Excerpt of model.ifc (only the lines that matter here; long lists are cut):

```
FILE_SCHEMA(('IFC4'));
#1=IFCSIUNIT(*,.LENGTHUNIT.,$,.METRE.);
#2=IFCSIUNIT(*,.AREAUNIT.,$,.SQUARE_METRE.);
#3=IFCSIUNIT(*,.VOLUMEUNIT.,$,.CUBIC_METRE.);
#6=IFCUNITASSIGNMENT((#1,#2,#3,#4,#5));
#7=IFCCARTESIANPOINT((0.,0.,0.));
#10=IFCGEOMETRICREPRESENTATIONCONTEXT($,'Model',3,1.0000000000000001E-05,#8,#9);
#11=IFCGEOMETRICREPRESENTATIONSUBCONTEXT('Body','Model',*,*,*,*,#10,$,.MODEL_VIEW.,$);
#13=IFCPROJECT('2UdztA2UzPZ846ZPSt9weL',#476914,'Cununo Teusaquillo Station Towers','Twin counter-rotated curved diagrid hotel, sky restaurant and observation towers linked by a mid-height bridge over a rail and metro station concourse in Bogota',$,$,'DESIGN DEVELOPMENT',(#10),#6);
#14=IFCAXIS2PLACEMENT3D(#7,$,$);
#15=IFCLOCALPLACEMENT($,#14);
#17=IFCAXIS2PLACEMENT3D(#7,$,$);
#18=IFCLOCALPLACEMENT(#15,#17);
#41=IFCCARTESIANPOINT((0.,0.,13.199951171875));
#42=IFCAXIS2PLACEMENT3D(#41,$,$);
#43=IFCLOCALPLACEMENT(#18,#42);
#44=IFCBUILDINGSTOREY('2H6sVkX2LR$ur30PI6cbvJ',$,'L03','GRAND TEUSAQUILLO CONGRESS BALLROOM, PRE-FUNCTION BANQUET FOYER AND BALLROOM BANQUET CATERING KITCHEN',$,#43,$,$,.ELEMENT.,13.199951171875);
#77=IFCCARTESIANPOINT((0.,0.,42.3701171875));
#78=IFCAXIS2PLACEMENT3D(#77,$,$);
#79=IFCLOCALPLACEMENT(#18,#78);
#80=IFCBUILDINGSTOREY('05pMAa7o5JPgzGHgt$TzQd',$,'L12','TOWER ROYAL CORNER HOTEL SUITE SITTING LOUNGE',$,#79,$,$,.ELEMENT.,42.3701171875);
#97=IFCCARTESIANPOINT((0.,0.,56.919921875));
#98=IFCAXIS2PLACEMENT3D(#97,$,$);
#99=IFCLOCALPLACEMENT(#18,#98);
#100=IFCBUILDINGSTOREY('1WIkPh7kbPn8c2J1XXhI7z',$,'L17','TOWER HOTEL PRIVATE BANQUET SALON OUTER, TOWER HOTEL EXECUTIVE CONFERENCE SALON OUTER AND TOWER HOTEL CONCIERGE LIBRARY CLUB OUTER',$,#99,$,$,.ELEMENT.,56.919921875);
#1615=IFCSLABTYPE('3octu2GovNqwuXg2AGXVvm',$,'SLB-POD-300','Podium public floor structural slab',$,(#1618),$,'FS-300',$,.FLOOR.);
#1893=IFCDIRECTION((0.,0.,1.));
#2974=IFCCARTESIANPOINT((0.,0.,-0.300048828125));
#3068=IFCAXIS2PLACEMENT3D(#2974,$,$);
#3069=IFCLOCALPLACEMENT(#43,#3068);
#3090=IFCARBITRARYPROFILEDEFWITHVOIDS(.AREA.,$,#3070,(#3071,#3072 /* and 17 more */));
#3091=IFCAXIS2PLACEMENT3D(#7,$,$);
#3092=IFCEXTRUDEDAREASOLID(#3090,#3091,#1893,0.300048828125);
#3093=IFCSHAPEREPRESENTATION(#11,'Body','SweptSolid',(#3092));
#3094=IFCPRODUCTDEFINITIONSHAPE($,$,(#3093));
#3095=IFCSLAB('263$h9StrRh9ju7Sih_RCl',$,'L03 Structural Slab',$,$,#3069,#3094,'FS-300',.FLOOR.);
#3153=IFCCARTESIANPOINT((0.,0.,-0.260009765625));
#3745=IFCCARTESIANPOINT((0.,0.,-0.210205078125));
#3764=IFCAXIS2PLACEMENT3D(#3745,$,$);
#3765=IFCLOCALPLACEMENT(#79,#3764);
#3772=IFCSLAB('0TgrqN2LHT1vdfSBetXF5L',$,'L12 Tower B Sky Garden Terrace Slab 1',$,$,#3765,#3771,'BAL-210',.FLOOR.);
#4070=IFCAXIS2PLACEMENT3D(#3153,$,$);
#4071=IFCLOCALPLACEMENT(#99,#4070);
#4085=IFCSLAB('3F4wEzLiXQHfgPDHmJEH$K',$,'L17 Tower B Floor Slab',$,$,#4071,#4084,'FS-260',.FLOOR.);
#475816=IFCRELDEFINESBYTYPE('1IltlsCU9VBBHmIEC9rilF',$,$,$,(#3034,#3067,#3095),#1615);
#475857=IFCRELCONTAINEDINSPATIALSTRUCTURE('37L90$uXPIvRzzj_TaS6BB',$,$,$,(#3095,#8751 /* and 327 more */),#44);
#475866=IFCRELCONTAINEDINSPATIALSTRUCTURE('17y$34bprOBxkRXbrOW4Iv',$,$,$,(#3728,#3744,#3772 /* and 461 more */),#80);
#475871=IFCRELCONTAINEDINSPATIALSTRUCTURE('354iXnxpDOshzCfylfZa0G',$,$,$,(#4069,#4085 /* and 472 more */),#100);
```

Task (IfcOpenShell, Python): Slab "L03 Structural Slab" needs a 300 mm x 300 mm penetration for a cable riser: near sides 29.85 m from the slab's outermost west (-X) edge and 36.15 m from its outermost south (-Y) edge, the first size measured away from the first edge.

```python
import numpy as np
import ifcopenshell
import ifcopenshell.api.feature
import ifcopenshell.api.geometry
import ifcopenshell.api.root
import ifcopenshell.geom
import ifcopenshell.util.placement
import ifcopenshell.util.representation
import ifcopenshell.util.shape
import ifcopenshell.util.unit

model = ifcopenshell.open("model.ifc")
unit_scale = ifcopenshell.util.unit.calculate_unit_scale(model)
settings = ifcopenshell.geom.settings()


def volume(element):
    """Net volume in cubic metres, openings subtracted."""
    shape = ifcopenshell.geom.create_shape(settings, element)
    return ifcopenshell.util.shape.get_volume(shape.geometry)


slab = model.by_id(3095)
before = volume(slab)

# Extent in the slab's own axes, in metres. The edges named are its -X and -Y sides.
slab_shape = ifcopenshell.geom.create_shape(settings, slab)
vertices = ifcopenshell.util.shape.get_vertices(slab_shape.geometry)
x_min, y_min, bottom = vertices.min(axis=0)
top = vertices[:, 2].max()

opening = ifcopenshell.api.root.create_entity(model, ifc_class="IfcOpeningElement", name="Cable riser opening", predefined_type="OPENING")
context = ifcopenshell.util.representation.get_context(model, "Model", "Body", "MODEL_VIEW")
width, depth = 0.3, 0.3
outline = [(0.0, 0.0), (width, 0.0), (width, depth), (0.0, depth), (0.0, 0.0)]
# Overshoot both faces by 50 mm so the cut is clean.
shape = ifcopenshell.api.geometry.add_slab_representation(
    model, context=context, depth=top - bottom + 0.1, polyline=outline
)
ifcopenshell.api.geometry.assign_representation(model, product=opening, representation=shape)

matrix = ifcopenshell.util.placement.get_local_placement(slab.ObjectPlacement)
matrix[:, 3] = matrix @ np.append(np.array([x_min + 29.85, y_min + 36.15, bottom - 0.05]) / unit_scale, 1.0)
ifcopenshell.api.geometry.edit_object_placement(model, product=opening, matrix=matrix, is_si=False)
ifcopenshell.api.feature.add_feature(model, feature=opening, element=slab)

after = volume(slab)

print(f"slab volume {before:.3f} -> {after:.3f} m3")

model.write("model_v2.ifc")
```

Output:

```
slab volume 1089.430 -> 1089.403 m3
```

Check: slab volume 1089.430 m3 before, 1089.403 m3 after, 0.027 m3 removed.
